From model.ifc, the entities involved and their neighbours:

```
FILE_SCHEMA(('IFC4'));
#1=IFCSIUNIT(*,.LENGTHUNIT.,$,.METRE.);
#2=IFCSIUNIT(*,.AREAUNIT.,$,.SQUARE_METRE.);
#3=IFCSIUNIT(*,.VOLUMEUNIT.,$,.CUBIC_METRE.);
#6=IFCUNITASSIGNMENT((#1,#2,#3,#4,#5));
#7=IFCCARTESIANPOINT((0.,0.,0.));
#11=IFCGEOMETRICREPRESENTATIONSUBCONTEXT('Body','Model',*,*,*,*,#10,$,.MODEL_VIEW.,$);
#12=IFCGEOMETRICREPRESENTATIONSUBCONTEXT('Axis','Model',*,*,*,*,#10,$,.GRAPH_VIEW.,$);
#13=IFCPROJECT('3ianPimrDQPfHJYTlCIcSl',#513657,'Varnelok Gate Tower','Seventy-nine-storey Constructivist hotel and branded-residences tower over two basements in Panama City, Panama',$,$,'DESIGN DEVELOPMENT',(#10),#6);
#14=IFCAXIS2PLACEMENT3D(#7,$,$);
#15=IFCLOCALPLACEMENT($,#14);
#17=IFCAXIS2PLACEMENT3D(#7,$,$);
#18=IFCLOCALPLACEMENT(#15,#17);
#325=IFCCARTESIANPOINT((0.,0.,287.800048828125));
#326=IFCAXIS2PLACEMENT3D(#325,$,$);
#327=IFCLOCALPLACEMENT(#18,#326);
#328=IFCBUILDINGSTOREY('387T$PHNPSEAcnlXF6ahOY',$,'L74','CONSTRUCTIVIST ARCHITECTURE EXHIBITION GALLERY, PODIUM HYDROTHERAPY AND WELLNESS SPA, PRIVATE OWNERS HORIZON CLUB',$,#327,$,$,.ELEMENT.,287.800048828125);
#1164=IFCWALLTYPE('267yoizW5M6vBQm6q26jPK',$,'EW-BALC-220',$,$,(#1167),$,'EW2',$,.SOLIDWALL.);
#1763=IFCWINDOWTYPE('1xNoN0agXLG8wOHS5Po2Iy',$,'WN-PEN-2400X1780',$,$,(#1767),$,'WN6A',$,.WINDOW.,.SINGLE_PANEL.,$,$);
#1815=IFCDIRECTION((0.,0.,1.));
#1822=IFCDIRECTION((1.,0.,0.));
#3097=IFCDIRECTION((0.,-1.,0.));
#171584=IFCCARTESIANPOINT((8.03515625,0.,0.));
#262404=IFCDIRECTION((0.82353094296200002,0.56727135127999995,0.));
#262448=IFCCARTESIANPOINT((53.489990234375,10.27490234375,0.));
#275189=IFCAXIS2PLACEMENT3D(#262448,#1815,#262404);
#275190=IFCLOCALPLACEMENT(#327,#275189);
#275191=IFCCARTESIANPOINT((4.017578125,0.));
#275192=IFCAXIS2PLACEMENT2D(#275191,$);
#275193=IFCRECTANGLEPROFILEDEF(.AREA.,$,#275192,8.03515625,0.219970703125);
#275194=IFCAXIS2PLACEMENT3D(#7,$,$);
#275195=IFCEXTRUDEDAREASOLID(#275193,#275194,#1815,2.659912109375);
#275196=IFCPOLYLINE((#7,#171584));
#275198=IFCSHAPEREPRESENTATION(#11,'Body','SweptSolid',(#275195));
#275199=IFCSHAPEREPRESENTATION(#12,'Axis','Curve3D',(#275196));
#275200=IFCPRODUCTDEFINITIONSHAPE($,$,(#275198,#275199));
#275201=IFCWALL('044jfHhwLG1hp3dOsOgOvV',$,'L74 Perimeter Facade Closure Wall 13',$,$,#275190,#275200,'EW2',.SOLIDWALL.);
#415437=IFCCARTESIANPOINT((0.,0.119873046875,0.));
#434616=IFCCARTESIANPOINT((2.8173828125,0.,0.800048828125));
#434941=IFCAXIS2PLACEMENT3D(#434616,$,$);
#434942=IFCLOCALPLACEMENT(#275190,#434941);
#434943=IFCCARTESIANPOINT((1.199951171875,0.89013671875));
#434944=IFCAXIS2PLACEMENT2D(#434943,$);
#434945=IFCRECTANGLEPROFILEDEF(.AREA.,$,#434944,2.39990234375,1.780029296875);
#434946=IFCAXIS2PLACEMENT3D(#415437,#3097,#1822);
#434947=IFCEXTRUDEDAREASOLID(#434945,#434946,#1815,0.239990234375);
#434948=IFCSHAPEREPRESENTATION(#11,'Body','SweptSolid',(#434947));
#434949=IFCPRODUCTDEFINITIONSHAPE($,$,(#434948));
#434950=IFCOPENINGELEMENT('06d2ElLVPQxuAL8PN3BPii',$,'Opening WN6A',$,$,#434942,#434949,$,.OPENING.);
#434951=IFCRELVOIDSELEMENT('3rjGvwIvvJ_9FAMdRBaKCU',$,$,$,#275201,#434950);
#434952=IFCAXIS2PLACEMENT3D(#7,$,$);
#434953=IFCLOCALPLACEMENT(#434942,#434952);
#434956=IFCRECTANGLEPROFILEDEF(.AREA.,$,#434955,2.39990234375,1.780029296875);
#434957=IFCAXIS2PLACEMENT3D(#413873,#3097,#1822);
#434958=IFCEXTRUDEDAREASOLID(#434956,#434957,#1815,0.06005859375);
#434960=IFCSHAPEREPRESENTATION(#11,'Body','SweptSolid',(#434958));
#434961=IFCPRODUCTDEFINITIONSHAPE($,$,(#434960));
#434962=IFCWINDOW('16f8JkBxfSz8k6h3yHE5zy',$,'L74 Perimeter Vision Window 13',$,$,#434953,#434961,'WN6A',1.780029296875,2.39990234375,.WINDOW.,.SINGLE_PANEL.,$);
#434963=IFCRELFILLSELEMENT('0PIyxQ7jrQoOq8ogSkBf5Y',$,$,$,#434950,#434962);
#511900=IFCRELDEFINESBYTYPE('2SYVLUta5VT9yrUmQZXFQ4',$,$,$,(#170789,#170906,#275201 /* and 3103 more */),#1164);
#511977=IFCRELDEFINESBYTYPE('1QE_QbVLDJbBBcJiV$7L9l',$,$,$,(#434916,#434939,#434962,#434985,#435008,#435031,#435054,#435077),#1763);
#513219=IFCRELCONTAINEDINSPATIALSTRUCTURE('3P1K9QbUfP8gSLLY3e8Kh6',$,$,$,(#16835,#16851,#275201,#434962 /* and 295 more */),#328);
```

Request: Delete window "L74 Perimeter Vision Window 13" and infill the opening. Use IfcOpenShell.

```python
import ifcopenshell
import ifcopenshell.api.feature
import ifcopenshell.api.root
import ifcopenshell.geom
import ifcopenshell.util.shape

model = ifcopenshell.open("model.ifc")
settings = ifcopenshell.geom.settings()


def volume(element):
    """Net volume in cubic metres, openings subtracted."""
    shape = ifcopenshell.geom.create_shape(settings, element)
    return ifcopenshell.util.shape.get_volume(shape.geometry)


window = model.by_guid("16f8JkBxfSz8k6h3yHE5zy")
opening = window.FillsVoids[0].RelatingOpeningElement
wall = opening.VoidsElements[0].RelatingBuildingElement
before = volume(wall)

ifcopenshell.api.root.remove_product(model, product=window)
ifcopenshell.api.feature.remove_feature(model, feature=opening)

after = volume(wall)

print(f"wall volume {before:.3f} -> {after:.3f} m3")

model.write("model_rev.ifc")
```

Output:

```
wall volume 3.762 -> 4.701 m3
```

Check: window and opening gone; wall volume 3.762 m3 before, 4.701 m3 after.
